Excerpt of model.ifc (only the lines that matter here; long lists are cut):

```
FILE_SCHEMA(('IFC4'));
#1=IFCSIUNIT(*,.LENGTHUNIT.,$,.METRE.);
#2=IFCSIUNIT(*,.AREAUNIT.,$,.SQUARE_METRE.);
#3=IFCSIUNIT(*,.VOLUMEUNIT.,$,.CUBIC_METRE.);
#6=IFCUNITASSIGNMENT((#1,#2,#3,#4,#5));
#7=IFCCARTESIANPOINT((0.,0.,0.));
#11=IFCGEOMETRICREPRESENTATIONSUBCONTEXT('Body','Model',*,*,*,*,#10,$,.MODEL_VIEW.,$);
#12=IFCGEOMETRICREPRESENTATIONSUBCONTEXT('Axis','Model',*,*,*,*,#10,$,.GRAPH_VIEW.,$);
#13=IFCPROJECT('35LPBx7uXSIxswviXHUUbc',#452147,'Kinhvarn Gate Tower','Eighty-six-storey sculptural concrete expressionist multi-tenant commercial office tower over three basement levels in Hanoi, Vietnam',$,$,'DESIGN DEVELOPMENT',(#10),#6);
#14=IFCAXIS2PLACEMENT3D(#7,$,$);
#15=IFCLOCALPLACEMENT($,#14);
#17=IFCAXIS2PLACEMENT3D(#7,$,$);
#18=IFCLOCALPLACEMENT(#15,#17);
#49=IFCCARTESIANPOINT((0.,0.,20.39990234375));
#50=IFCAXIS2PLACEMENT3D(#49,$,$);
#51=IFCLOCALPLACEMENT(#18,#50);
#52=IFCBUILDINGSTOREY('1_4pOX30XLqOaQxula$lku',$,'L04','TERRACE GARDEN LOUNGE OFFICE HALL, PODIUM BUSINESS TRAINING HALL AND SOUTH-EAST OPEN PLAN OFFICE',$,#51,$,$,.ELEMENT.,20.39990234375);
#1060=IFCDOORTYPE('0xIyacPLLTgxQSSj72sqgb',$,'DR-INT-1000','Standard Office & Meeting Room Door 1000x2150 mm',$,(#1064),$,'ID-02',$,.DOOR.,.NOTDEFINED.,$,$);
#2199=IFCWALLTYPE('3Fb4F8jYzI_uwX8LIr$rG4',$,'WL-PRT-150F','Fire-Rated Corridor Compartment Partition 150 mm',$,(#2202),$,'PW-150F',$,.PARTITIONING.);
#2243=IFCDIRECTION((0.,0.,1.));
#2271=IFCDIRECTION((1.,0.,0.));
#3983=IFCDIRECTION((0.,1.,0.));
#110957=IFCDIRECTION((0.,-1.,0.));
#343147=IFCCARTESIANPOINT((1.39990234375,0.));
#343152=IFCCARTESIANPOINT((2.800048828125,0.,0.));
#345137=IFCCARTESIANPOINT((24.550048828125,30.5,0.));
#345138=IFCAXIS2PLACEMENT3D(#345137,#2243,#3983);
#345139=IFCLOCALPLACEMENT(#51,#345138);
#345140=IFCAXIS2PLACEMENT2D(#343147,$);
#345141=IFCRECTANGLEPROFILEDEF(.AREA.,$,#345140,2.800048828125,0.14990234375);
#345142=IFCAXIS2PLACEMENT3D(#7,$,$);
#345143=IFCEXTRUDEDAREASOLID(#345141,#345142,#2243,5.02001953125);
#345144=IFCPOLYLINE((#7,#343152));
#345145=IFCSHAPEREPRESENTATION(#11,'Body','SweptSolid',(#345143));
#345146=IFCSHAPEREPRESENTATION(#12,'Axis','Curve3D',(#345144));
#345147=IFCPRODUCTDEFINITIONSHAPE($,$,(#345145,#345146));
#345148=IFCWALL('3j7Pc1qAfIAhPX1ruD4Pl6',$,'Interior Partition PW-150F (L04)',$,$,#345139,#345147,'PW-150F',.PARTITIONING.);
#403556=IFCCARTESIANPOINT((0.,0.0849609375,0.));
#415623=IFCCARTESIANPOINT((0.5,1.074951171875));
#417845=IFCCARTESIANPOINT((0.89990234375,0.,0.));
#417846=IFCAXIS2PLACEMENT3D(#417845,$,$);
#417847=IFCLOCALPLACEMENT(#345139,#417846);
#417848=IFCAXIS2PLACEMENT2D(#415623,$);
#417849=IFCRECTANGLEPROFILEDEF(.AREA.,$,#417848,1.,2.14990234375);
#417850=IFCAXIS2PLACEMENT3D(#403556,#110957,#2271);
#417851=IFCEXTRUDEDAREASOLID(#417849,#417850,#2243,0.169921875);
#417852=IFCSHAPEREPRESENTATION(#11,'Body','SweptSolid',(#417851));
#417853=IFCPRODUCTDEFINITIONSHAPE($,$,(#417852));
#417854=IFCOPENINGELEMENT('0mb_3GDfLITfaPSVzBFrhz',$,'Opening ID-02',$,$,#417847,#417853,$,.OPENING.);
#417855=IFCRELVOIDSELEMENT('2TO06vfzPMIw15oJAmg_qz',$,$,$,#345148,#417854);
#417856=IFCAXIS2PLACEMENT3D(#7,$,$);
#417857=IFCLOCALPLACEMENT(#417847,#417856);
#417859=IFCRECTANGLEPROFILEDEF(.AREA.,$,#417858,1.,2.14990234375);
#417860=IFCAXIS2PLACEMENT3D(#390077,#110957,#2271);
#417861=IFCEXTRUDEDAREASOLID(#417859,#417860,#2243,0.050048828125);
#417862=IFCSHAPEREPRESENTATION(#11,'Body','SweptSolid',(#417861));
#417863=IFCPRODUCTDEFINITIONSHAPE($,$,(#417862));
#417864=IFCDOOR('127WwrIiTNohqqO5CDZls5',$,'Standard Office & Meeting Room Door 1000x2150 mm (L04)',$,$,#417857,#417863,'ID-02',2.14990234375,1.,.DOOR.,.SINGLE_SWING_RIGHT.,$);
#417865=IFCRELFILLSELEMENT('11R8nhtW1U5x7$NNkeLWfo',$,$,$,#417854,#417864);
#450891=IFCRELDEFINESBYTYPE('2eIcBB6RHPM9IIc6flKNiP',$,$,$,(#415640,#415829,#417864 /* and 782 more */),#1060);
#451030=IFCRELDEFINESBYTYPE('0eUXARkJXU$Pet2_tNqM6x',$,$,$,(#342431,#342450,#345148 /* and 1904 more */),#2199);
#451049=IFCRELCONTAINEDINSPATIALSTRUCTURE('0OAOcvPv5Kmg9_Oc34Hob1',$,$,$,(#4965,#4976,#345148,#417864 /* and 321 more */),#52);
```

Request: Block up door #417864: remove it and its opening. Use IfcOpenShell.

```python
import ifcopenshell
import ifcopenshell.api.feature
import ifcopenshell.api.root
import ifcopenshell.geom
import ifcopenshell.util.shape

model = ifcopenshell.open("model.ifc")
settings = ifcopenshell.geom.settings()


def volume(element):
    """Net volume in cubic metres, openings subtracted."""
    shape = ifcopenshell.geom.create_shape(settings, element)
    return ifcopenshell.util.shape.get_volume(shape.geometry)


door = model.by_guid("127WwrIiTNohqqO5CDZls5")
opening = door.FillsVoids[0].RelatingOpeningElement
wall = opening.VoidsElements[0].RelatingBuildingElement
before = volume(wall)

ifcopenshell.api.root.remove_product(model, product=door)
ifcopenshell.api.feature.remove_feature(model, feature=opening)

after = volume(wall)

print(f"wall volume {before:.3f} -> {after:.3f} m3")

model.write("model_edited.ifc")
```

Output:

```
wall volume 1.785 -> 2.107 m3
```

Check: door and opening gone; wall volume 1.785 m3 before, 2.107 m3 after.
